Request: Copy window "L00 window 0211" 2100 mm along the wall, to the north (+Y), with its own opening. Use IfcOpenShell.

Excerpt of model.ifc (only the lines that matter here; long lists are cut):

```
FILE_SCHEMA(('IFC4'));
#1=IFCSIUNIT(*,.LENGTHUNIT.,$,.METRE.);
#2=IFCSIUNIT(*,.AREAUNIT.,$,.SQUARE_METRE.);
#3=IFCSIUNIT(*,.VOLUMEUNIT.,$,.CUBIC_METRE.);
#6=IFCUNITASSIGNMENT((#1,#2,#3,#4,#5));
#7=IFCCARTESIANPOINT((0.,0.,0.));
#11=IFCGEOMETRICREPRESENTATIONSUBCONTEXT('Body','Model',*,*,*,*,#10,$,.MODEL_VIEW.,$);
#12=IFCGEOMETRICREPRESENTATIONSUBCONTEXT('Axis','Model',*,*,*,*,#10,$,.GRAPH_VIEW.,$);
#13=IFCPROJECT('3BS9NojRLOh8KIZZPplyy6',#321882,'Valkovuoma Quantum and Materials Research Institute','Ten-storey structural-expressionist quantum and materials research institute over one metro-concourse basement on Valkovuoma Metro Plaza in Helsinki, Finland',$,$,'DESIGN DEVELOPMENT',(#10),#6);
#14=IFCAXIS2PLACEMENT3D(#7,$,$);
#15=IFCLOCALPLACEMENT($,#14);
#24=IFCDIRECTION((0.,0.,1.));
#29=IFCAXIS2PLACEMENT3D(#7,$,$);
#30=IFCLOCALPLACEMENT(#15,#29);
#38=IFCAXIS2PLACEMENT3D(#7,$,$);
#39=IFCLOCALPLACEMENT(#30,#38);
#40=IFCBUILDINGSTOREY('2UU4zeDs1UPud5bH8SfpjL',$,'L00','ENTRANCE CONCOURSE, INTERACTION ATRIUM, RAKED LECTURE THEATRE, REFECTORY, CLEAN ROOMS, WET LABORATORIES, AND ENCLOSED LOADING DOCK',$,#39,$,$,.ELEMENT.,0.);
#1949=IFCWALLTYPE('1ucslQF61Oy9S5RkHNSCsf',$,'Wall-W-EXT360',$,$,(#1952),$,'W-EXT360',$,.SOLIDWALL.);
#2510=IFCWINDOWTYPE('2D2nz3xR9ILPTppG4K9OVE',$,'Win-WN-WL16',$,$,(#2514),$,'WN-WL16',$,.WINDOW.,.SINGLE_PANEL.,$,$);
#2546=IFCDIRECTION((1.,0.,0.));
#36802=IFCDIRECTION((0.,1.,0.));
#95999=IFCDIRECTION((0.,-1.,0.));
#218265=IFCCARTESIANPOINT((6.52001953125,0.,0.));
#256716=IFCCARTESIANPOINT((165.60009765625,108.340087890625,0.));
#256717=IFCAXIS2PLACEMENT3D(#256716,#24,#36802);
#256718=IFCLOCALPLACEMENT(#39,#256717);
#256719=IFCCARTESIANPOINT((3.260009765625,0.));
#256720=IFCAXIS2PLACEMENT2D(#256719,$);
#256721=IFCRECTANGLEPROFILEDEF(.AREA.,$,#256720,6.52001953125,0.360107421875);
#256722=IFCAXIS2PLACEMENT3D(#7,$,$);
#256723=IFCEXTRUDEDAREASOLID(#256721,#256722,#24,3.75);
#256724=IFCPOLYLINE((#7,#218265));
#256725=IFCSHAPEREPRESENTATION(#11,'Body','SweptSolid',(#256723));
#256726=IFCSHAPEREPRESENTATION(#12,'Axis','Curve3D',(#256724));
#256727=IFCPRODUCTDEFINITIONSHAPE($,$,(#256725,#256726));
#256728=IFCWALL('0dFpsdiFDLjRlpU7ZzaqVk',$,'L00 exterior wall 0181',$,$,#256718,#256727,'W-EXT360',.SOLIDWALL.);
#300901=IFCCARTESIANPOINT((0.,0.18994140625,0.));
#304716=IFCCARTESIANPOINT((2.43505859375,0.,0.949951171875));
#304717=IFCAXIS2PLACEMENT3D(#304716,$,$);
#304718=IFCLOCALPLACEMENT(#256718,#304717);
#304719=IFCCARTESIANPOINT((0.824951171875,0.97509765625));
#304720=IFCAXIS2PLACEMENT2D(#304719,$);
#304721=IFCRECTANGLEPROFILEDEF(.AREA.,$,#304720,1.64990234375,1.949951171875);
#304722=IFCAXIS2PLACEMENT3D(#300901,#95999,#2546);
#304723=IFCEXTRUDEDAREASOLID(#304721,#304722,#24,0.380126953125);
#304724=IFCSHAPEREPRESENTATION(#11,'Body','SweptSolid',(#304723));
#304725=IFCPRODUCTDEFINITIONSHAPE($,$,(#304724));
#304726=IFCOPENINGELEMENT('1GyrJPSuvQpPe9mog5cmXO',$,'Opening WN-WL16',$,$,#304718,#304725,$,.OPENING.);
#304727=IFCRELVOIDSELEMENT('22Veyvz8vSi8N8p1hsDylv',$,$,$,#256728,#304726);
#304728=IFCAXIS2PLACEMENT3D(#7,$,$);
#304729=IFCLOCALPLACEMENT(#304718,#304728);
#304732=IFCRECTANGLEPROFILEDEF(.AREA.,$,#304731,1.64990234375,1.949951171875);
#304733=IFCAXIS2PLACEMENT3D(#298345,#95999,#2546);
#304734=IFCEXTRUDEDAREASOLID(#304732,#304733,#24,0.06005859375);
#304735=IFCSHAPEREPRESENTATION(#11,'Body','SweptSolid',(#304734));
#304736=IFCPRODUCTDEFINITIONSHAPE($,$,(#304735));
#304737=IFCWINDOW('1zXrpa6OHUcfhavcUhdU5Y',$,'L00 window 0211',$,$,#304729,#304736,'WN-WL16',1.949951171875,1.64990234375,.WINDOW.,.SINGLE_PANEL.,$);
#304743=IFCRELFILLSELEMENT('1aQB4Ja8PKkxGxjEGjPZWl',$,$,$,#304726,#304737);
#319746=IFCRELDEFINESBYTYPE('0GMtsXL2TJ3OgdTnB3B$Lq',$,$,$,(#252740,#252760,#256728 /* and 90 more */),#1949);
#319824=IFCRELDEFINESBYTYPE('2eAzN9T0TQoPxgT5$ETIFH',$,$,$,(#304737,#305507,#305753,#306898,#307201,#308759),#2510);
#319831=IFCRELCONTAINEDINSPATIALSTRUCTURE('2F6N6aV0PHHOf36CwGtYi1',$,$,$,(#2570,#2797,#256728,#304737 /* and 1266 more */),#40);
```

```python
import ifcopenshell
import ifcopenshell.api.feature
import ifcopenshell.api.geometry
import ifcopenshell.api.root
import ifcopenshell.geom
import ifcopenshell.util.element
import ifcopenshell.util.placement
import ifcopenshell.util.shape
import ifcopenshell.util.unit

model = ifcopenshell.open("model.ifc")
unit_scale = ifcopenshell.util.unit.calculate_unit_scale(model)
settings = ifcopenshell.geom.settings()


def volume(element):
    """Net volume in cubic metres, openings subtracted."""
    shape = ifcopenshell.geom.create_shape(settings, element)
    return ifcopenshell.util.shape.get_volume(shape.geometry)


window = model.by_id(304737)
opening = window.FillsVoids[0].RelatingOpeningElement
wall = opening.VoidsElements[0].RelatingBuildingElement
before = volume(wall)
shift = ifcopenshell.util.placement.get_local_placement(wall.ObjectPlacement)[:3, 0] * 2.1 / unit_scale

# copy_class copies the void relationship, type, container and properties, but no geometry.
new_opening = ifcopenshell.api.root.copy_class(model, product=opening)
new_opening.Representation = ifcopenshell.util.element.copy_deep(
    model, opening.Representation, exclude=["IfcGeometricRepresentationContext", "IfcRepresentationMap"]
)
new_window = ifcopenshell.api.root.copy_class(model, product=window)
new_window.Representation = ifcopenshell.util.element.copy_deep(
    model, window.Representation, exclude=["IfcGeometricRepresentationContext", "IfcRepresentationMap"]
)
new_window.Tag = None
ifcopenshell.api.feature.add_filling(model, opening=new_opening, element=new_window)

for old, new in ((opening, new_opening), (window, new_window)):
    matrix = ifcopenshell.util.placement.get_local_placement(old.ObjectPlacement)
    matrix[:3, 3] += shift
    ifcopenshell.api.geometry.edit_object_placement(model, product=new, matrix=matrix, is_si=False)

after = volume(wall)

print(f"wall volume {before:.3f} -> {after:.3f} m3")

model.write("model-out.ifc")
```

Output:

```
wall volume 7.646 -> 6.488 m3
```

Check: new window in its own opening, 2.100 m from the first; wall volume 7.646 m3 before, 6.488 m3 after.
